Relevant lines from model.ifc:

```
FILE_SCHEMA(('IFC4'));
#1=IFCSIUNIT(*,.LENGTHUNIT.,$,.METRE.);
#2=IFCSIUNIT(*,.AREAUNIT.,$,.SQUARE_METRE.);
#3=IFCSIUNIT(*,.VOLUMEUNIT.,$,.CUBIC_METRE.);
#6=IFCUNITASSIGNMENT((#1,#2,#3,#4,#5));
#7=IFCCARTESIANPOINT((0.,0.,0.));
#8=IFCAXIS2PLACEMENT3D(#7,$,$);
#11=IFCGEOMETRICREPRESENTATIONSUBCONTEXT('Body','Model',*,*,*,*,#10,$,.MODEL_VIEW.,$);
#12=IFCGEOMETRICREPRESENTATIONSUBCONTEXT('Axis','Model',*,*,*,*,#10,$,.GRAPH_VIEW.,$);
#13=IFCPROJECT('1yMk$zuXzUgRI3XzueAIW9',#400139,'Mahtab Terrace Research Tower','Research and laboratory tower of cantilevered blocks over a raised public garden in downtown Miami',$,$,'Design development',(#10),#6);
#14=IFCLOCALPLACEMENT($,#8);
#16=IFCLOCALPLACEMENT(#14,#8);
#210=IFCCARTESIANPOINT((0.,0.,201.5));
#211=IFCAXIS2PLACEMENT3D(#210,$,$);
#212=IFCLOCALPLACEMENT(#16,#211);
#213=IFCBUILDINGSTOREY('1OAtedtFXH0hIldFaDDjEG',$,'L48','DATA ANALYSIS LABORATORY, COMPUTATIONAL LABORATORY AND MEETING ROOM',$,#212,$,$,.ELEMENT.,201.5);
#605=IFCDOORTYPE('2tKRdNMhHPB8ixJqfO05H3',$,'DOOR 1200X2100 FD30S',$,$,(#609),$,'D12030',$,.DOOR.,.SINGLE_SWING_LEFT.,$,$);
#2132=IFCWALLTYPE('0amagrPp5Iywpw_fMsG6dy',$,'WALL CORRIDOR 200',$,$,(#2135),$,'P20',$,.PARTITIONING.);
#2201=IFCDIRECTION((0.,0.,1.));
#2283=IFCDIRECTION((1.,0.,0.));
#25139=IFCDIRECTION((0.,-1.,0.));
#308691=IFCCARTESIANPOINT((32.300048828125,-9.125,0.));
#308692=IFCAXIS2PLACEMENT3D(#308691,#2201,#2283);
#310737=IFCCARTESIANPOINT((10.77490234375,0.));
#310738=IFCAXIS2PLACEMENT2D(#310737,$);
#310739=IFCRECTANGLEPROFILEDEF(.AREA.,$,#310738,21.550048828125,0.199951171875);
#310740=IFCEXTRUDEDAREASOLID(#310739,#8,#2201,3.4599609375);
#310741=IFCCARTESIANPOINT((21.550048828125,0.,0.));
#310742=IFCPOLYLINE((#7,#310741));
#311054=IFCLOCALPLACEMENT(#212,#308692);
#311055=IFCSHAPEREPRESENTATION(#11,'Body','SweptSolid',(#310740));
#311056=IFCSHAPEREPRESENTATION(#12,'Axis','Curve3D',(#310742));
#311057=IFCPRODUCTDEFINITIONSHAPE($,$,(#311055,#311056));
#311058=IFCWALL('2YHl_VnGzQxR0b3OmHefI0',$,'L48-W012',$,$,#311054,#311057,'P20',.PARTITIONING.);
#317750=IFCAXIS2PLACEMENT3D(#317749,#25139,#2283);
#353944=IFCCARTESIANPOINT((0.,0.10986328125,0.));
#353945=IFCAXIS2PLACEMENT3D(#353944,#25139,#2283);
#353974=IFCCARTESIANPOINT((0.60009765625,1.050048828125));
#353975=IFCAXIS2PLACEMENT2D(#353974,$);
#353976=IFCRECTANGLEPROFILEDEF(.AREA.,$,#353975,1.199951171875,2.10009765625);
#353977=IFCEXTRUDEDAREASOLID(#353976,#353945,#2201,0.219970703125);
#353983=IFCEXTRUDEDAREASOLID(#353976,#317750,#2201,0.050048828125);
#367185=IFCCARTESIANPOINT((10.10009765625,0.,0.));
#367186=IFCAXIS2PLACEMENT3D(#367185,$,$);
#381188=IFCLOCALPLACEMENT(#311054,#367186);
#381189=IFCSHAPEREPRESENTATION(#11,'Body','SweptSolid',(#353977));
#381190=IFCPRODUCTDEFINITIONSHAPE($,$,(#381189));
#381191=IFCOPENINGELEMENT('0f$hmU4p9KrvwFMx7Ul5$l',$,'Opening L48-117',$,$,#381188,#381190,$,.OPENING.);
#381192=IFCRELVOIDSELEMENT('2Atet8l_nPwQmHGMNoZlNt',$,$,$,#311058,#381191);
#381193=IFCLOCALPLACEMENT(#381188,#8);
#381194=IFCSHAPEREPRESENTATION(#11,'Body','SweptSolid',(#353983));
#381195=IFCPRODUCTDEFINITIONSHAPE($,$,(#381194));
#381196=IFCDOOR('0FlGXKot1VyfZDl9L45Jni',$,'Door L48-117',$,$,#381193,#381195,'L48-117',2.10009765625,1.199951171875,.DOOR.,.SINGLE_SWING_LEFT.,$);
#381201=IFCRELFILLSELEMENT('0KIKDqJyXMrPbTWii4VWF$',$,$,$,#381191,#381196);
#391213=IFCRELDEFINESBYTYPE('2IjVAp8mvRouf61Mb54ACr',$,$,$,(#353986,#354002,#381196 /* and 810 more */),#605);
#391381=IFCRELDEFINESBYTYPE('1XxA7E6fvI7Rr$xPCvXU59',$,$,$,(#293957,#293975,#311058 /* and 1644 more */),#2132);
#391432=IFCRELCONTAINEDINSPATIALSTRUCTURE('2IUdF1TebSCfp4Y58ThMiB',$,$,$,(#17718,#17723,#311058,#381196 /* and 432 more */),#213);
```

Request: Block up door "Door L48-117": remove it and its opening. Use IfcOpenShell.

```python
import ifcopenshell
import ifcopenshell.api.feature
import ifcopenshell.api.root
import ifcopenshell.geom
import ifcopenshell.util.shape

model = ifcopenshell.open("model.ifc")
settings = ifcopenshell.geom.settings()


def volume(element):
    """Net volume in cubic metres, openings subtracted."""
    shape = ifcopenshell.geom.create_shape(settings, element)
    return ifcopenshell.util.shape.get_volume(shape.geometry)


door = model.by_id(381196)
opening = door.FillsVoids[0].RelatingOpeningElement
wall = opening.VoidsElements[0].RelatingBuildingElement
before = volume(wall)

ifcopenshell.api.root.remove_product(model, product=door)
ifcopenshell.api.feature.remove_feature(model, feature=opening)

after = volume(wall)

print(f"wall volume {before:.3f} -> {after:.3f} m3")

model.write("model-out.ifc")
```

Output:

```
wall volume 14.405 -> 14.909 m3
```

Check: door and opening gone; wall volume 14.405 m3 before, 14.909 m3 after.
